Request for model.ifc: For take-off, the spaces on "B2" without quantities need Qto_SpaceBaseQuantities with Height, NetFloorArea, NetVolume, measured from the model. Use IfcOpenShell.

First a look at what the model holds.

```python
import ifcopenshell
import ifcopenshell.util.element
import ifcopenshell.util.unit

model = ifcopenshell.open("model.ifc")
print(model.schema)
for unit_type in ("LENGTHUNIT", "AREAUNIT", "VOLUMEUNIT"):
    print(unit_type, ifcopenshell.util.unit.calculate_unit_scale(model, unit_type))
storey = next(s for s in model.by_type("IfcBuildingStorey") if s.Name == "B2")
spaces = [e for e in ifcopenshell.util.element.get_decomposition(storey) if e.is_a("IfcSpace")]
for e in sorted(spaces, key=lambda e: e.id()):
    print(e.id(), e.is_a(), e.Name, list(ifcopenshell.util.element.get_psets(e, qtos_only=True)), sep=" | ")
```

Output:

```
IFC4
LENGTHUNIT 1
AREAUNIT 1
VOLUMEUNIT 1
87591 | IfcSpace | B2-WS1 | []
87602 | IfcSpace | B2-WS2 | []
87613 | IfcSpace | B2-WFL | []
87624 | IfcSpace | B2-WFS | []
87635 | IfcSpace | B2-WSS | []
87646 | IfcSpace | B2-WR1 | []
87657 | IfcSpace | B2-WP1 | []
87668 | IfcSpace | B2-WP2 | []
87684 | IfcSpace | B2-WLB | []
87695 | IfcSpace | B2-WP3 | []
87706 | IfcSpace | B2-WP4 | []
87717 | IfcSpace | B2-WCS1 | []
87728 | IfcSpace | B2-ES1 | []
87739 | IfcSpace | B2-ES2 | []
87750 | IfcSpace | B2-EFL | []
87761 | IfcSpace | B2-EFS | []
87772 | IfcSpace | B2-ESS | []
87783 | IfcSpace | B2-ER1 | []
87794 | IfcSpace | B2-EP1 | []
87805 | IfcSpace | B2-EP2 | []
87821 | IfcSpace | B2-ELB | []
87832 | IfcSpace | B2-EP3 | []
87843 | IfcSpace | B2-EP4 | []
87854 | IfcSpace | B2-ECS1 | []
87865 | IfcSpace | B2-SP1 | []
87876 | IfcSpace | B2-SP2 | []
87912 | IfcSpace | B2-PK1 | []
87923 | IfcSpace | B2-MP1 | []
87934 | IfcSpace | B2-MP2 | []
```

```python
import ifcopenshell
import ifcopenshell.api.pset
import ifcopenshell.geom
import ifcopenshell.util.element
import ifcopenshell.util.shape
import ifcopenshell.util.unit

model = ifcopenshell.open("model.ifc")
unit_scale = ifcopenshell.util.unit.calculate_unit_scale(model)
area_scale = ifcopenshell.util.unit.calculate_unit_scale(model, "AREAUNIT")
volume_scale = ifcopenshell.util.unit.calculate_unit_scale(model, "VOLUMEUNIT")
settings = ifcopenshell.geom.settings()

storey = next(s for s in model.by_type("IfcBuildingStorey") if s.Name == "B2")
spaces = [e for e in ifcopenshell.util.element.get_decomposition(storey) if e.is_a("IfcSpace")]

for e in sorted(spaces, key=lambda e: e.id()):
    if ifcopenshell.util.element.get_psets(e, qtos_only=True, should_inherit=False):
        continue
    # Geometry comes back in metres, in the element's own axes.
    shape = ifcopenshell.geom.create_shape(settings, e)
    values = {
        "Height": ifcopenshell.util.shape.get_z(shape.geometry) / unit_scale,
        "NetFloorArea": ifcopenshell.util.shape.get_footprint_area(shape.geometry) / area_scale,
        "NetVolume": ifcopenshell.util.shape.get_volume(shape.geometry) / volume_scale,
    }
    qto = ifcopenshell.api.pset.add_qto(model, product=e, name="Qto_SpaceBaseQuantities")
    ifcopenshell.api.pset.edit_qto(model, qto=qto, properties=values)
    print(e.id(), {k: round(v, 3) for k, v in values.items()})

model.write("model_v2.ifc")
```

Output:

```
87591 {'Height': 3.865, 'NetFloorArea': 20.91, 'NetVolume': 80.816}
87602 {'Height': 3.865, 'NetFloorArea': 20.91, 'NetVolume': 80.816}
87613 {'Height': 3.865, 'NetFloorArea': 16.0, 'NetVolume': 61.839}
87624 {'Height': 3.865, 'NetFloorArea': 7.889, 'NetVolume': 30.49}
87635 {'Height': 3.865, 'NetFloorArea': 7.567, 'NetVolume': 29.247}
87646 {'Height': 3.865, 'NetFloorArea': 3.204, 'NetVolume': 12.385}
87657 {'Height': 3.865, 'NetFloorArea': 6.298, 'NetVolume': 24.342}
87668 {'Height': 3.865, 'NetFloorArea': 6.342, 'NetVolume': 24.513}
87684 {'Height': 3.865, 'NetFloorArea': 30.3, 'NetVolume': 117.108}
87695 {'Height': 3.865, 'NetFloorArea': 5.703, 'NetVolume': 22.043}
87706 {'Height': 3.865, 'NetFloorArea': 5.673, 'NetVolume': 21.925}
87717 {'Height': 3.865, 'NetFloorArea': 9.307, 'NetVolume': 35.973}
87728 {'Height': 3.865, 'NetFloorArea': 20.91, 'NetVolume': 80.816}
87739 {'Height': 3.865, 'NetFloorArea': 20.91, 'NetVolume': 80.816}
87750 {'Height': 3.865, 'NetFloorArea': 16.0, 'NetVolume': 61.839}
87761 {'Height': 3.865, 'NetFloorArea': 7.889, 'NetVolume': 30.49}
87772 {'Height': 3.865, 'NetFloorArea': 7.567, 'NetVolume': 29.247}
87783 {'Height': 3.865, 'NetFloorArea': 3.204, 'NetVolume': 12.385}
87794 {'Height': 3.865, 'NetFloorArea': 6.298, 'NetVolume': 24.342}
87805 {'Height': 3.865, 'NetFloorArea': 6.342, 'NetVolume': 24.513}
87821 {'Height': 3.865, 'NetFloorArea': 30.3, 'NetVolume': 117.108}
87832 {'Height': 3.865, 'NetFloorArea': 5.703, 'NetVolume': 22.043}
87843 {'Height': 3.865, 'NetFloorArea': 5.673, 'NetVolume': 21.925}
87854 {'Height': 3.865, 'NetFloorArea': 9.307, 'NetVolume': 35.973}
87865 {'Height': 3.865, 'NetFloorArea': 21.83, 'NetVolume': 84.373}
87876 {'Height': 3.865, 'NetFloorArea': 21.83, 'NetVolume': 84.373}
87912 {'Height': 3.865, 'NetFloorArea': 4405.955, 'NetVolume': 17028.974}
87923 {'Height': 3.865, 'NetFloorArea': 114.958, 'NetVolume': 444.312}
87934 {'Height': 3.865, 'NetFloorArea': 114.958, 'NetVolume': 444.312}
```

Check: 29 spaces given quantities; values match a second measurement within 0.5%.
